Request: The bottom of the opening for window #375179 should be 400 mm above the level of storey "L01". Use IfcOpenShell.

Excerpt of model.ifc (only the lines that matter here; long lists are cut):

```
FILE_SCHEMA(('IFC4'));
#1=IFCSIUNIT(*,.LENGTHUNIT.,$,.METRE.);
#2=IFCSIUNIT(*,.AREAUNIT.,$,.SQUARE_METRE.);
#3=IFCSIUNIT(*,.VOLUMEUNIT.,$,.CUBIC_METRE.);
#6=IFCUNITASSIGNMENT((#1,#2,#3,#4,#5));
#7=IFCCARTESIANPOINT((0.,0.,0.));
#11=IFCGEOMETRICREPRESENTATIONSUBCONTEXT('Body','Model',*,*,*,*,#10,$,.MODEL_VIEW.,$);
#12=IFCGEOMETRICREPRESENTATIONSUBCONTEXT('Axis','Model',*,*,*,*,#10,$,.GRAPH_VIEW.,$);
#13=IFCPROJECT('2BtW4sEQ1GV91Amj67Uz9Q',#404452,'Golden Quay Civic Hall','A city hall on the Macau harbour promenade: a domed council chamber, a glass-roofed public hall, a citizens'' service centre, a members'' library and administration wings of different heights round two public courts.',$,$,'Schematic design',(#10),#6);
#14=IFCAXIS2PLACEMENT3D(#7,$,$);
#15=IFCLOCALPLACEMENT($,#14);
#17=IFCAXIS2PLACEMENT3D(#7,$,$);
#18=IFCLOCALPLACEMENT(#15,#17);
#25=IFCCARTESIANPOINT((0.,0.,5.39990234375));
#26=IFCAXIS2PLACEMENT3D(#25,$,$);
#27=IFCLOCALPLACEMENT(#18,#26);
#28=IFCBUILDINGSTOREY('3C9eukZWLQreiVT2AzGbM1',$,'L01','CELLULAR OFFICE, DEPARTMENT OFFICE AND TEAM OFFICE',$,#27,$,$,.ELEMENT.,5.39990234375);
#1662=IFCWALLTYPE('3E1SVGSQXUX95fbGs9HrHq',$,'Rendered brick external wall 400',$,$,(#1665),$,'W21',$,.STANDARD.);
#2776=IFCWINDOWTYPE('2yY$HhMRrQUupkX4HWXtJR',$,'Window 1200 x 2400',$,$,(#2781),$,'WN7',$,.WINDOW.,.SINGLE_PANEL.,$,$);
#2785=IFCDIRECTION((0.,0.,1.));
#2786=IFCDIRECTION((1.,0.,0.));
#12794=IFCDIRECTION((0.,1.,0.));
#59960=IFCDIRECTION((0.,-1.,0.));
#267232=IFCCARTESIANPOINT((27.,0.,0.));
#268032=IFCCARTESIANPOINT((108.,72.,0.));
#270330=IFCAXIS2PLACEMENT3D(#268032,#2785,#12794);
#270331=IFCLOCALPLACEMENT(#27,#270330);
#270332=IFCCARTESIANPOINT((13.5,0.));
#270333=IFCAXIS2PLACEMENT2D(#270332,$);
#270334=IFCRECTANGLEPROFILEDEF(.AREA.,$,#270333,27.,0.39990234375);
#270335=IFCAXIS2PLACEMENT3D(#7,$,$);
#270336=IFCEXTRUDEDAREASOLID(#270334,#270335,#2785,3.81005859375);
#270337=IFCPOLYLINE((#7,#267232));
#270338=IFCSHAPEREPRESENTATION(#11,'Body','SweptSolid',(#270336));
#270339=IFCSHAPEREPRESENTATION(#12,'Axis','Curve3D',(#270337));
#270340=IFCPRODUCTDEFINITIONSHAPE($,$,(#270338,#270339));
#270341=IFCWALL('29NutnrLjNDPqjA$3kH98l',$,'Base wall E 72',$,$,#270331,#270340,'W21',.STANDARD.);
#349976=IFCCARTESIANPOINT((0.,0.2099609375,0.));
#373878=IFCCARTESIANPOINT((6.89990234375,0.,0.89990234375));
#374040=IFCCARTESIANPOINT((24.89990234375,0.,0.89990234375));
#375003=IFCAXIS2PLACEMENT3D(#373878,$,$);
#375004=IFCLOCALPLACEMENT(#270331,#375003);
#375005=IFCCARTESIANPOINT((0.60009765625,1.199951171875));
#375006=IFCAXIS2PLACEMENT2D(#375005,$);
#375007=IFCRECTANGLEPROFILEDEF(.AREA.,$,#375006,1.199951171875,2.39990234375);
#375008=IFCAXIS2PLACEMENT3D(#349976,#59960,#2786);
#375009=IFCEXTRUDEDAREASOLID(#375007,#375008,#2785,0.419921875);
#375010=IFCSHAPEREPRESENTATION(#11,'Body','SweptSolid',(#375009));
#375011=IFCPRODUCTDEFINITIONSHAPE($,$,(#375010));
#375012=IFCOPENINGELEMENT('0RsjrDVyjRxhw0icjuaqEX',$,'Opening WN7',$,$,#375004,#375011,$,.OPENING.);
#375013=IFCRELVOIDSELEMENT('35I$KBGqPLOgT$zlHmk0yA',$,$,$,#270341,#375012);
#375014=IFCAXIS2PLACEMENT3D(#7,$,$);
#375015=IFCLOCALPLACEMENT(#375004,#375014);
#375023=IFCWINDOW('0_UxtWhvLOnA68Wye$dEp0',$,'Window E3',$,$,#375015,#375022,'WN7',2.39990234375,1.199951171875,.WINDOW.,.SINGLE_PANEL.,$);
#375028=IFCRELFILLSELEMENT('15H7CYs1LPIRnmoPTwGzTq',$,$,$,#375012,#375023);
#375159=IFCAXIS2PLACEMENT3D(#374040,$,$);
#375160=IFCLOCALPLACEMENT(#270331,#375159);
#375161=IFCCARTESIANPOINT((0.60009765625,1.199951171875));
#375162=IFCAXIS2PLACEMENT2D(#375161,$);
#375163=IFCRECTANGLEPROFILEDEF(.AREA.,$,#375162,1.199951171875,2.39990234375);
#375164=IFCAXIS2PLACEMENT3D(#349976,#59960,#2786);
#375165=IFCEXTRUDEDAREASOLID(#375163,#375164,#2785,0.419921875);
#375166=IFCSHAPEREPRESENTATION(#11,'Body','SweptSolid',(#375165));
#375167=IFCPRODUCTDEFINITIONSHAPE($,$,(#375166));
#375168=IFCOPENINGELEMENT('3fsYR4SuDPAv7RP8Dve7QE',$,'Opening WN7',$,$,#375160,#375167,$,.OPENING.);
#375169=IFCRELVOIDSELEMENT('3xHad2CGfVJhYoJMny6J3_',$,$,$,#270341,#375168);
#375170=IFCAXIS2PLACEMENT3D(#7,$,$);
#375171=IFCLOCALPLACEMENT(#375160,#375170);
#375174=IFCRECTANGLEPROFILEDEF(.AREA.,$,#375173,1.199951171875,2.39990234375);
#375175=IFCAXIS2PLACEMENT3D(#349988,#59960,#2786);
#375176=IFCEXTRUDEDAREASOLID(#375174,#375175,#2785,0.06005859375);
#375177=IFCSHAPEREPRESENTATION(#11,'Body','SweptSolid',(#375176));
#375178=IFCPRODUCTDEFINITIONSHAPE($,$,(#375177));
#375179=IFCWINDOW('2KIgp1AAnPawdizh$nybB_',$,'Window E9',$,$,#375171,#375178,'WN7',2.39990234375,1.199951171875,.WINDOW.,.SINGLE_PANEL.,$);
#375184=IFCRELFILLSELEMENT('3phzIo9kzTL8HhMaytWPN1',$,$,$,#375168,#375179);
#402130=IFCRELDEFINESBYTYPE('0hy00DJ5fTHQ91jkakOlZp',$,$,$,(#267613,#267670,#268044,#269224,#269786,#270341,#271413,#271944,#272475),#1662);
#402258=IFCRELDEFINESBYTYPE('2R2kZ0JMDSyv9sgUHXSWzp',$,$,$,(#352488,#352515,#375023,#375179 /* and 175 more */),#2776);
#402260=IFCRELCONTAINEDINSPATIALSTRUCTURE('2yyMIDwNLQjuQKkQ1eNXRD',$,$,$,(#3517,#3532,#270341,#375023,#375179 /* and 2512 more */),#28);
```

```python
import numpy as np
import ifcopenshell
import ifcopenshell.api.geometry
import ifcopenshell.geom
import ifcopenshell.util.element
import ifcopenshell.util.placement
import ifcopenshell.util.shape
import ifcopenshell.util.unit

model = ifcopenshell.open("model.ifc")
unit_scale = ifcopenshell.util.unit.calculate_unit_scale(model)

window = model.by_guid("2KIgp1AAnPawdizh$nybB_")
opening = window.FillsVoids[0].RelatingOpeningElement
storey = ifcopenshell.util.element.get_container(window, ifc_class="IfcBuildingStorey")
level = ifcopenshell.util.placement.get_local_placement(storey.ObjectPlacement)[2, 3]

# The opening's origin need not be at the sill, so measure its lowest point.
shape = ifcopenshell.geom.create_shape(ifcopenshell.geom.settings(), opening)
bottom = ifcopenshell.util.shape.get_shape_bottom_elevation(shape, shape.geometry) / unit_scale
dz = level + 0.4 - bottom

shift = np.array([0.0, 0.0, dz])
# The window is placed relative to its opening, so it follows when the opening moves.
matrix = ifcopenshell.util.placement.get_local_placement(opening.ObjectPlacement)
matrix[:3, 3] += shift
ifcopenshell.api.geometry.edit_object_placement(
    model, product=opening, matrix=matrix, is_si=False, should_transform_children=True
)

print(f"moved by {dz * unit_scale:+.3f} m")

model.write("model_updated.ifc")
```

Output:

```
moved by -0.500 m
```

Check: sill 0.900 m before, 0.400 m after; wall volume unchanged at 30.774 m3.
